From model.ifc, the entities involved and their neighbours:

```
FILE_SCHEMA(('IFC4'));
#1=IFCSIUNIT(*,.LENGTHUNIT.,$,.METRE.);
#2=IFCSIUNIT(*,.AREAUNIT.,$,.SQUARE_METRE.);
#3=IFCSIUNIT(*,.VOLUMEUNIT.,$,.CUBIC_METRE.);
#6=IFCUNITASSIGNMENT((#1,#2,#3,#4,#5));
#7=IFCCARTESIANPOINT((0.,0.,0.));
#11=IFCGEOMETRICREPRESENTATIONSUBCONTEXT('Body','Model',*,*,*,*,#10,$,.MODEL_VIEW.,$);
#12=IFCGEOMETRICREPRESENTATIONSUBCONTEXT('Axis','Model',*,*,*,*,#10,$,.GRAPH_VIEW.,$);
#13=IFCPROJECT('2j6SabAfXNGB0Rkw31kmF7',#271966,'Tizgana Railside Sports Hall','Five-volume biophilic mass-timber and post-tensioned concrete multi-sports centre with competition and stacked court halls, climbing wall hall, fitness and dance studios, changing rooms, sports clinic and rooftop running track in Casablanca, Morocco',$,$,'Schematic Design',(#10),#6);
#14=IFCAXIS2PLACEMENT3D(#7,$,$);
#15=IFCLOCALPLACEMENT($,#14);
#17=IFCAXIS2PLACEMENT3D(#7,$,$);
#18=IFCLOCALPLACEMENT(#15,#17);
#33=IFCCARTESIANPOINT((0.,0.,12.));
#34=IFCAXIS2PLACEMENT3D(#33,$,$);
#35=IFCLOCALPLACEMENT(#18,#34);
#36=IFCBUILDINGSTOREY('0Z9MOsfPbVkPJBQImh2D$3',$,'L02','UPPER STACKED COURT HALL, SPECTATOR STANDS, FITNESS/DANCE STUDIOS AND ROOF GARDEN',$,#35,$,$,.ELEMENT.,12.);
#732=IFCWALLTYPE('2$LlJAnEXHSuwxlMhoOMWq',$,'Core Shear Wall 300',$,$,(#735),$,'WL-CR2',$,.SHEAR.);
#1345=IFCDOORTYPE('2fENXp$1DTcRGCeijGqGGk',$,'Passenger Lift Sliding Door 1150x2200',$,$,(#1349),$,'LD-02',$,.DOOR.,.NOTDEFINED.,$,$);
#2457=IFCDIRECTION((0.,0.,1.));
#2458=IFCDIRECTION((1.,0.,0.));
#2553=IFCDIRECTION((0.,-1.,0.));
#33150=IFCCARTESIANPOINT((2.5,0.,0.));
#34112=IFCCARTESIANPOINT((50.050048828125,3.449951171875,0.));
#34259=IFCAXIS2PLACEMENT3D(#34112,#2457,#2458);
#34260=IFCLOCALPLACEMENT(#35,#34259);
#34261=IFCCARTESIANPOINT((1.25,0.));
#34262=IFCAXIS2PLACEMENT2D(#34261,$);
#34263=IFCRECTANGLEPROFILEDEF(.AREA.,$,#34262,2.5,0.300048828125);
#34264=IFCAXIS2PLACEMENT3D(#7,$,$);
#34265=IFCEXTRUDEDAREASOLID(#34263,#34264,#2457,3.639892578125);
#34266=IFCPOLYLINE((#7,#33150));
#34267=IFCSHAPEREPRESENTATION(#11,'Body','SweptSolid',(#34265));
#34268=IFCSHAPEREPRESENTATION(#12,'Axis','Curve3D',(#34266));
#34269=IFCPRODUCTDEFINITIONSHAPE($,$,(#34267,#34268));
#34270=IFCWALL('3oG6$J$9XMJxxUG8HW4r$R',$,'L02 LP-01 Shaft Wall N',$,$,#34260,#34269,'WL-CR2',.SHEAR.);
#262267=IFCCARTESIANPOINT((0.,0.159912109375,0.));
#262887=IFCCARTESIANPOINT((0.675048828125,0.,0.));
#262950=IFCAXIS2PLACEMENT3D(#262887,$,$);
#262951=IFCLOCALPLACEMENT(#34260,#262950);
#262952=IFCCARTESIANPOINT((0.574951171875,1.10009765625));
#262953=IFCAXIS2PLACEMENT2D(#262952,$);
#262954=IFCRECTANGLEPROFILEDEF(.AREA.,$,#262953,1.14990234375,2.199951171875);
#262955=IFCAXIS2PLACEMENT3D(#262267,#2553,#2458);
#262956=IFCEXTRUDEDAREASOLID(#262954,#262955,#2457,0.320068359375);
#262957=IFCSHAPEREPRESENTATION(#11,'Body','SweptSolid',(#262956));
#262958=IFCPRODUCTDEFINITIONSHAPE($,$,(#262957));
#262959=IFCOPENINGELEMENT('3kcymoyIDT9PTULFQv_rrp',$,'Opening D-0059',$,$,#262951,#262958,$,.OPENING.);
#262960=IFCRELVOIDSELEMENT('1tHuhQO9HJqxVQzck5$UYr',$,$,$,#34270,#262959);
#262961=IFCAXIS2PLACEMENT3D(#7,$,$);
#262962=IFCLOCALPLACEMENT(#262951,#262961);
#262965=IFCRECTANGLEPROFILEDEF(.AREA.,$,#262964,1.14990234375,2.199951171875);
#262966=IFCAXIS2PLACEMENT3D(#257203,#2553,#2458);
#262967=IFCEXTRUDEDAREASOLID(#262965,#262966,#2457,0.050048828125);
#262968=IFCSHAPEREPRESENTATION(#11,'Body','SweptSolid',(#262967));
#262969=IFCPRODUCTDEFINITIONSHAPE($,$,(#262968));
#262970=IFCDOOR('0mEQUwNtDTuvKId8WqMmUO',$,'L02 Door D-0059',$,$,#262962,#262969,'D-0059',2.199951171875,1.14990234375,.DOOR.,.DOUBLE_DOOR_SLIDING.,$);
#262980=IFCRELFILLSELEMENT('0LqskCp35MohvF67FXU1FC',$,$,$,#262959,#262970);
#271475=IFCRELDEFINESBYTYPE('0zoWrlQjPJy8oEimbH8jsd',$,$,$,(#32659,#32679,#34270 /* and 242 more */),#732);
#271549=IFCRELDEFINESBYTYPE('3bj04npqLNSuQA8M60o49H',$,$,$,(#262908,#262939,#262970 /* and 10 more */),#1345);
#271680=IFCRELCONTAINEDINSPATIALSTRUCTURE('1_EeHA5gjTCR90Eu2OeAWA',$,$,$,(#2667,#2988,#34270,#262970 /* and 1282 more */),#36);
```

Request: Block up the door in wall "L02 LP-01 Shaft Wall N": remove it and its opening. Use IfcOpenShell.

```python
import ifcopenshell
import ifcopenshell.api.feature
import ifcopenshell.api.root
import ifcopenshell.geom
import ifcopenshell.util.shape

model = ifcopenshell.open("model.ifc")
settings = ifcopenshell.geom.settings()


def volume(element):
    """Net volume in cubic metres, openings subtracted."""
    shape = ifcopenshell.geom.create_shape(settings, element)
    return ifcopenshell.util.shape.get_volume(shape.geometry)


door = model.by_id(262970)
opening = door.FillsVoids[0].RelatingOpeningElement
wall = opening.VoidsElements[0].RelatingBuildingElement
before = volume(wall)

ifcopenshell.api.root.remove_product(model, product=door)
ifcopenshell.api.feature.remove_feature(model, feature=opening)

after = volume(wall)

print(f"wall volume {before:.3f} -> {after:.3f} m3")

model.write("model-out.ifc")
```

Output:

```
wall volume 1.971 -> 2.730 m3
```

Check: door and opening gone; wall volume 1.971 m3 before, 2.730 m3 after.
